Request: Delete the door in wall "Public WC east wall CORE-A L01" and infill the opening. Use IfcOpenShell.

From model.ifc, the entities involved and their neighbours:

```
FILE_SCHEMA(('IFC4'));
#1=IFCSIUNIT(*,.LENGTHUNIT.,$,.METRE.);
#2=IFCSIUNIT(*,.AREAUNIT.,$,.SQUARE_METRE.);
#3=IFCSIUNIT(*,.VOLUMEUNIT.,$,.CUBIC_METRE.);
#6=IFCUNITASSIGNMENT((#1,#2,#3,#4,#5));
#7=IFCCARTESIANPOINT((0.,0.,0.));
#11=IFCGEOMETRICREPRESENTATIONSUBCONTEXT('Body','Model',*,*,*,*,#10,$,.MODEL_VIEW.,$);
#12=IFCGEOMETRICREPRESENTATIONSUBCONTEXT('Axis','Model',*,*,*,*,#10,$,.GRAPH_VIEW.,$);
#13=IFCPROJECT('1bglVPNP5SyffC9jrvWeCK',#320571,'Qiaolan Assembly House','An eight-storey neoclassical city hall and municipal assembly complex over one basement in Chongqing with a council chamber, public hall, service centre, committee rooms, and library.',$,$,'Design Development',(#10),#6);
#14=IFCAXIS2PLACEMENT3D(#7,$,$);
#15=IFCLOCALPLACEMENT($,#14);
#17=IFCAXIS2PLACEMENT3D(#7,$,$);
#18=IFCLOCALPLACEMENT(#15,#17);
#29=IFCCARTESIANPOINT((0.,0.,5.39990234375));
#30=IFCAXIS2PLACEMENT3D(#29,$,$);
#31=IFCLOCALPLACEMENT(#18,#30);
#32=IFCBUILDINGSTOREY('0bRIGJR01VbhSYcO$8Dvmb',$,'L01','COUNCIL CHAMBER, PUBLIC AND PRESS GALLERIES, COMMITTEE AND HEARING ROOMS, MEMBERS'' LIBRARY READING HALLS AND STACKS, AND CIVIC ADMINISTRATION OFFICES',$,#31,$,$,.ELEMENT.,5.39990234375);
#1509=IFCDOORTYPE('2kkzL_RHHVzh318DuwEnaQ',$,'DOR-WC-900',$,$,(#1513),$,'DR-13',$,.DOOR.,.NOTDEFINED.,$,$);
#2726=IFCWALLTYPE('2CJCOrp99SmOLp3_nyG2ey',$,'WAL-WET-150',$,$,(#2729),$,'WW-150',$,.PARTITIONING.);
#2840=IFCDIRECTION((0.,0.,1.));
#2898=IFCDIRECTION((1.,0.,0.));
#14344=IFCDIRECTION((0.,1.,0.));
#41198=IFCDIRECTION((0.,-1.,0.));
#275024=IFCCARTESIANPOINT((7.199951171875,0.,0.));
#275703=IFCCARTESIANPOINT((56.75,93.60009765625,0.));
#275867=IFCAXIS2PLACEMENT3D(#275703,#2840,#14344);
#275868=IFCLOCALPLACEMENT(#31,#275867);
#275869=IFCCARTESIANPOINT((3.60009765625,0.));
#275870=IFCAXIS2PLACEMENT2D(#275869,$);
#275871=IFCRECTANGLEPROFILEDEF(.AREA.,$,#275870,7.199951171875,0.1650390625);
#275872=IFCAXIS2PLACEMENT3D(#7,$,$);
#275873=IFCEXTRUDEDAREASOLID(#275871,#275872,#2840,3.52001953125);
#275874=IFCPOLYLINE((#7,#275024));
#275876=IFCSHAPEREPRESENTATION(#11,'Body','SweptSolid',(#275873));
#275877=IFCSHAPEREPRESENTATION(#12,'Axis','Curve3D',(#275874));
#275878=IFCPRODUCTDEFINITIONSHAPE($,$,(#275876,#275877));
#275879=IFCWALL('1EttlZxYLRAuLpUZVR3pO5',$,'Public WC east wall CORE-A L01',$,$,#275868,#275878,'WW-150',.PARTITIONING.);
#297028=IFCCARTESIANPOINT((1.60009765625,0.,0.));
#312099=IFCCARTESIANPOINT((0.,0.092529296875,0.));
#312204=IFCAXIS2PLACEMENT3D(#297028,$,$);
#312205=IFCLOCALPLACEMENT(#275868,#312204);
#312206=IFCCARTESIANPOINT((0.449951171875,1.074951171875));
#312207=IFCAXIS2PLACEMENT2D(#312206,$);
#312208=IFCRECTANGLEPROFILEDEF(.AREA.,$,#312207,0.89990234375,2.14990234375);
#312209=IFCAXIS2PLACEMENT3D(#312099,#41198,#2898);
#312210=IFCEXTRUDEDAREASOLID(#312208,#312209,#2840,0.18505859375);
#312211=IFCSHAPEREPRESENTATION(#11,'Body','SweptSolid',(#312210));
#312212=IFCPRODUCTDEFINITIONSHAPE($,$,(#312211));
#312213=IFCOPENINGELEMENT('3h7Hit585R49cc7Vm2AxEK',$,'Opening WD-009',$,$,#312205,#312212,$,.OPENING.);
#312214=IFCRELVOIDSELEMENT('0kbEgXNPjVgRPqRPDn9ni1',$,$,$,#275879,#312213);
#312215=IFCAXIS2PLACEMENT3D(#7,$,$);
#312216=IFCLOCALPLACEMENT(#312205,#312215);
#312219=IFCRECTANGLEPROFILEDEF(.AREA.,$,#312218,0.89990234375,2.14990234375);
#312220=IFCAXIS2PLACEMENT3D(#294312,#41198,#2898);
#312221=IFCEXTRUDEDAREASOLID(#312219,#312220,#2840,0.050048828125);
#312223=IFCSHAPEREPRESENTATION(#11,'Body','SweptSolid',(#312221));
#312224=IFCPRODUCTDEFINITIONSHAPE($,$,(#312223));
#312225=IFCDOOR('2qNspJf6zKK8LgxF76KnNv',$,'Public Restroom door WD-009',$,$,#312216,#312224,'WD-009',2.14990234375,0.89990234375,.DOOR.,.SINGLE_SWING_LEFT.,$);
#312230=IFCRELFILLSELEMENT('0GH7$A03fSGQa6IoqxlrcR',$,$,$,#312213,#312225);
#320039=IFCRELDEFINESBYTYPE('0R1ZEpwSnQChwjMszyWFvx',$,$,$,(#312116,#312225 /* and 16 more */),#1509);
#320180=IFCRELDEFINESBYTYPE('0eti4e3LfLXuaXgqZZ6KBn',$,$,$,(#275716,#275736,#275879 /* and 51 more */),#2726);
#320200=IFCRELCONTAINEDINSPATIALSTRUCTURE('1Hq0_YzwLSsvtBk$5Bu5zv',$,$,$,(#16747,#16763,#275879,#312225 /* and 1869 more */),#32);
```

```python
import ifcopenshell
import ifcopenshell.api.feature
import ifcopenshell.api.root
import ifcopenshell.geom
import ifcopenshell.util.shape

model = ifcopenshell.open("model.ifc")
settings = ifcopenshell.geom.settings()


def volume(element):
    """Net volume in cubic metres, openings subtracted."""
    shape = ifcopenshell.geom.create_shape(settings, element)
    return ifcopenshell.util.shape.get_volume(shape.geometry)


door = model.by_guid("2qNspJf6zKK8LgxF76KnNv")
opening = door.FillsVoids[0].RelatingOpeningElement
wall = opening.VoidsElements[0].RelatingBuildingElement
before = volume(wall)

ifcopenshell.api.root.remove_product(model, product=door)
ifcopenshell.api.feature.remove_feature(model, feature=opening)

after = volume(wall)

print(f"wall volume {before:.3f} -> {after:.3f} m3")

model.write("model_v2.ifc")
```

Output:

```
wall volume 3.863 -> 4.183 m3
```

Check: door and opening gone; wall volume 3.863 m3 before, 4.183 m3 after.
